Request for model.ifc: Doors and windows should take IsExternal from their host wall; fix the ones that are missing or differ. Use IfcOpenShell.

First a look at what the model holds.

```python
import ifcopenshell
import ifcopenshell.util.element

model = ifcopenshell.open("model.ifc")
print(model.schema)
seen = {}
for e in model.by_type("IfcDoor") + model.by_type("IfcWindow"):
    if not e.FillsVoids:
        continue
    host = e.FillsVoids[0].RelatingOpeningElement.VoidsElements[0].RelatingBuildingElement
    own = ifcopenshell.util.element.get_pset(e, f"Pset_{e.is_a()[3:].removesuffix('StandardCase')}Common", "IsExternal")
    wall = ifcopenshell.util.element.get_pset(host, "Pset_WallCommon", "IsExternal")
    seen[e.is_a(), own, wall] = seen.get((e.is_a(), own, wall), 0) + 1
for (cls, own, wall), count in sorted(seen.items(), key=str):
    print(count, cls, "IsExternal:", own, "| host wall:", wall)
```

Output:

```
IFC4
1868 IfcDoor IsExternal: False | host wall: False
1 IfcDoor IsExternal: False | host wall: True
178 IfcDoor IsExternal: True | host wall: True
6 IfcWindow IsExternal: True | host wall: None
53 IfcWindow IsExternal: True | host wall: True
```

```python
import ifcopenshell
import ifcopenshell.api.pset
import ifcopenshell.util.element

model = ifcopenshell.open("model.ifc")

count = 0
for ifc_class, pset_name in (("IfcDoor", "Pset_DoorCommon"), ("IfcWindow", "Pset_WindowCommon")):
    for e in model.by_type(ifc_class):
        if not e.FillsVoids:
            continue
        host = e.FillsVoids[0].RelatingOpeningElement.VoidsElements[0].RelatingBuildingElement
        external = ifcopenshell.util.element.get_pset(host, "Pset_WallCommon", "IsExternal")
        if external is None or ifcopenshell.util.element.get_pset(e, pset_name, "IsExternal") == external:
            continue
        pset = ifcopenshell.api.pset.add_pset(model, product=e, name=pset_name)
        ifcopenshell.api.pset.edit_pset(model, pset=pset, properties={"IsExternal": external})
        count += 1

print(count, "updated")

model.write("model-out.ifc")
```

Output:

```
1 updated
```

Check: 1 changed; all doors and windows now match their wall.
